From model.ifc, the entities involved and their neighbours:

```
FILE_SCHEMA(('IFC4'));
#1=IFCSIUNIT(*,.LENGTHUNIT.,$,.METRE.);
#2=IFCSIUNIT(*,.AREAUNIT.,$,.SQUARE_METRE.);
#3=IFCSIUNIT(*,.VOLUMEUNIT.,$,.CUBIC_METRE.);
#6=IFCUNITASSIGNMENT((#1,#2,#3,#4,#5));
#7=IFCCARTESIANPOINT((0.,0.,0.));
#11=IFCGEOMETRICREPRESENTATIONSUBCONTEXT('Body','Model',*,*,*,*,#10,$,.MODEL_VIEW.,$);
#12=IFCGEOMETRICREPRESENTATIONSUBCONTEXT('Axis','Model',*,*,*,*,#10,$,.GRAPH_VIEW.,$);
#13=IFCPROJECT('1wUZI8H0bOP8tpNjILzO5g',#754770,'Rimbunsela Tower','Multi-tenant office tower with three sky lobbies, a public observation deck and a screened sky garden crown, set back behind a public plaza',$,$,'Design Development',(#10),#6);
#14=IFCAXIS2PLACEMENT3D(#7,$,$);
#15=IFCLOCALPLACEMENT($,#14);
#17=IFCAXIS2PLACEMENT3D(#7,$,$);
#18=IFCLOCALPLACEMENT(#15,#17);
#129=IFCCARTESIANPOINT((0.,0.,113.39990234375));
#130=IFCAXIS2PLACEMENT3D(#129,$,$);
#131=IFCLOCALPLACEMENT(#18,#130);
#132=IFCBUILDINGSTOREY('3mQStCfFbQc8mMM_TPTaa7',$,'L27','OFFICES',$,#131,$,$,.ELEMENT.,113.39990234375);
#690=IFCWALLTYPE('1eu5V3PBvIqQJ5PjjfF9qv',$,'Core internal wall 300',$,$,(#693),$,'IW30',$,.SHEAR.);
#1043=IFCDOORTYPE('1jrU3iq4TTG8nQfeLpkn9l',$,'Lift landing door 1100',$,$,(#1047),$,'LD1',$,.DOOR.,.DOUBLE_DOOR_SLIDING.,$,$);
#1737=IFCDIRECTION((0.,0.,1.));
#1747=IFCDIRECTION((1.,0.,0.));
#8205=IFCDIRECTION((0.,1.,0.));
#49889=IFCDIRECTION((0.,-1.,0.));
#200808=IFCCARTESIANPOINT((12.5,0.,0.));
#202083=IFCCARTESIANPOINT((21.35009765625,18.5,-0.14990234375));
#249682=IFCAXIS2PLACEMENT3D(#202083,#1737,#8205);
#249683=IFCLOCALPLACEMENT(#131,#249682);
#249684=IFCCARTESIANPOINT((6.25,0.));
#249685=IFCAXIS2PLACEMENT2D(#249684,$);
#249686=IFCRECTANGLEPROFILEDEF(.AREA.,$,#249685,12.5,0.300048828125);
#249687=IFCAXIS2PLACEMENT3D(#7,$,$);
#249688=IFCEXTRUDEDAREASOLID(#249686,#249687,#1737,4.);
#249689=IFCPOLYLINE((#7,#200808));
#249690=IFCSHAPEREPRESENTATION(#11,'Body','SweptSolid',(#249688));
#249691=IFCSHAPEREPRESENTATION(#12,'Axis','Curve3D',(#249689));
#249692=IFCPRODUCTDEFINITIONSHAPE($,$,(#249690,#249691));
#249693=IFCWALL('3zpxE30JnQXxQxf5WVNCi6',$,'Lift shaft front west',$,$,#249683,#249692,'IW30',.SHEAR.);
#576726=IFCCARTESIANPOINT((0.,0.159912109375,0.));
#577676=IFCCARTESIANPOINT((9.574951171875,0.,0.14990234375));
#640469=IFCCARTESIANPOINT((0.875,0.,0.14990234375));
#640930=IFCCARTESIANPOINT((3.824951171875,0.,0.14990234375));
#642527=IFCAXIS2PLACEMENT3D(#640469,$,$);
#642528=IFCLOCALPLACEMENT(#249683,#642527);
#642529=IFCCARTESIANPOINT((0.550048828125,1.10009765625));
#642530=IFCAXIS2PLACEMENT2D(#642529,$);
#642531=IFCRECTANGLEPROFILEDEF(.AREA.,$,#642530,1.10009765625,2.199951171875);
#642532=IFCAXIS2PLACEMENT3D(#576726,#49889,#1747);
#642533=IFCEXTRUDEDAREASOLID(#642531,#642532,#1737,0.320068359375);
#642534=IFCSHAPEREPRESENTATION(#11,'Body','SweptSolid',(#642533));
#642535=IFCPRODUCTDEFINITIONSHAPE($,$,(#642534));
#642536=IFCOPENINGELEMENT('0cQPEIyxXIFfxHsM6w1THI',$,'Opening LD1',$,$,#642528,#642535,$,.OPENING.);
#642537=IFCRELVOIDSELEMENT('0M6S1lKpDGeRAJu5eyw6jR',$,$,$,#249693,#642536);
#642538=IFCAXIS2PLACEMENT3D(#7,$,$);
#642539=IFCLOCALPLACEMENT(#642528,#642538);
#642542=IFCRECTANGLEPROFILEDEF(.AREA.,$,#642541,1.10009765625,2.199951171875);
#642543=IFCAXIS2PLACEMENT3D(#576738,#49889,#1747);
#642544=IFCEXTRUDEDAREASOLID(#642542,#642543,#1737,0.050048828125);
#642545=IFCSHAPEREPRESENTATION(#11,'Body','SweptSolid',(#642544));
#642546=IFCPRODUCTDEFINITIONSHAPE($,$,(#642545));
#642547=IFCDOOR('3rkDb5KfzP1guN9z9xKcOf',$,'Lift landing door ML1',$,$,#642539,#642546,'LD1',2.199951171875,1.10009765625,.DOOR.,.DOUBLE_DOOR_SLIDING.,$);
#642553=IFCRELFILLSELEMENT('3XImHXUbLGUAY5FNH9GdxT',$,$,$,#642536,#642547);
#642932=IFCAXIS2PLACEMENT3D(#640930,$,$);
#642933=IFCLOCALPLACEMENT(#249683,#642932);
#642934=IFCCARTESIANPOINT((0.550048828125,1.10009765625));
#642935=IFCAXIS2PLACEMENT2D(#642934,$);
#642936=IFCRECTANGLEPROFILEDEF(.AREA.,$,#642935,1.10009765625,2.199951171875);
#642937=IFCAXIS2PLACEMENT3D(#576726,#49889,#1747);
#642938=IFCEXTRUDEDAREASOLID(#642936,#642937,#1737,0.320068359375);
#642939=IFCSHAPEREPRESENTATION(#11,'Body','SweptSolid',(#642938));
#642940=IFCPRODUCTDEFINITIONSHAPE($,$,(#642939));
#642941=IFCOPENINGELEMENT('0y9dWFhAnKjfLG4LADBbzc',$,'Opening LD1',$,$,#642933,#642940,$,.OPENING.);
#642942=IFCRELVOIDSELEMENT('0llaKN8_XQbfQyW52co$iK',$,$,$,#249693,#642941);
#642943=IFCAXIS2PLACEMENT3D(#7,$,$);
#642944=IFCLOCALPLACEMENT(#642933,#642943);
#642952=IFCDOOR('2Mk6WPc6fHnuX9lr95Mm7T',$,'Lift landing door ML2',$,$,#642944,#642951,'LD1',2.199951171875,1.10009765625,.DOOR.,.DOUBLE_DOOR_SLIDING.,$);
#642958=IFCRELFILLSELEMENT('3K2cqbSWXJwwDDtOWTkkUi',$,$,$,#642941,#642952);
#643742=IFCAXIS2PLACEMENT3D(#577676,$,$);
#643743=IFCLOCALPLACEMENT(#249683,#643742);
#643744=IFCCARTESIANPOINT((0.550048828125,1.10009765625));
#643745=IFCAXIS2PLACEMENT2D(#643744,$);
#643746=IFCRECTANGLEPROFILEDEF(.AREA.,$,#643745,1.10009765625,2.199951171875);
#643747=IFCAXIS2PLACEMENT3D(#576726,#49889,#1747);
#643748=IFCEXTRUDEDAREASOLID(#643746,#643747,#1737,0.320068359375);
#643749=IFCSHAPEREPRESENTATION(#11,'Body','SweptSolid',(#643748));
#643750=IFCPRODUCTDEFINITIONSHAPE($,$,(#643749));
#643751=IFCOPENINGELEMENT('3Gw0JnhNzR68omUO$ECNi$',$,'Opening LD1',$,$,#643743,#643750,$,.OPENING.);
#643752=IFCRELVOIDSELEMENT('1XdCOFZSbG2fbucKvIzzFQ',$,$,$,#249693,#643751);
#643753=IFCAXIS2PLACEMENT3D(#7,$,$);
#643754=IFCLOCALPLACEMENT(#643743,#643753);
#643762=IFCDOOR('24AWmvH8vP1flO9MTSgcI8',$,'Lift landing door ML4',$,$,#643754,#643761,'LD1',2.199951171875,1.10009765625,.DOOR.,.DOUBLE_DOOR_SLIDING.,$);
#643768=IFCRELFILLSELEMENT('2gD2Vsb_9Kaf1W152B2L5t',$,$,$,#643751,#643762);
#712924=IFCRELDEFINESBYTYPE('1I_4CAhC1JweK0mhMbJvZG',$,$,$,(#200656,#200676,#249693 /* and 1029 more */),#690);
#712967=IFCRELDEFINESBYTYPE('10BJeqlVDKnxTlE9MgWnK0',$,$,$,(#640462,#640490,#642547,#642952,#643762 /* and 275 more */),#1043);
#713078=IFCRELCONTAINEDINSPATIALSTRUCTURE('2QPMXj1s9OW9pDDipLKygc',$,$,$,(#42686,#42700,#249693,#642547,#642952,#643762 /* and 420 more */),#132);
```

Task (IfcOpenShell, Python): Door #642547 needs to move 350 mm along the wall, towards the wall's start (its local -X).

```python
import ifcopenshell
import ifcopenshell.api.geometry
import ifcopenshell.util.placement
import ifcopenshell.util.unit

model = ifcopenshell.open("model.ifc")
unit_scale = ifcopenshell.util.unit.calculate_unit_scale(model)

door = model.by_guid("3rkDb5KfzP1guN9z9xKcOf")
opening = door.FillsVoids[0].RelatingOpeningElement
wall = opening.VoidsElements[0].RelatingBuildingElement

wall_matrix = ifcopenshell.util.placement.get_local_placement(wall.ObjectPlacement)
shift = wall_matrix[:3, 0] * -0.35 / unit_scale
before = ifcopenshell.util.placement.get_local_placement(door.ObjectPlacement)[:3, 3].copy()

# The door is placed relative to its opening, so it follows when the opening moves.
matrix = ifcopenshell.util.placement.get_local_placement(opening.ObjectPlacement)
matrix[:3, 3] += shift
ifcopenshell.api.geometry.edit_object_placement(
    model, product=opening, matrix=matrix, is_si=False, should_transform_children=True
)

after = ifcopenshell.util.placement.get_local_placement(door.ObjectPlacement)[:3, 3]
print("door moved by", (after - before).round(3) + 0.0)

model.write("model_edited.ifc")
```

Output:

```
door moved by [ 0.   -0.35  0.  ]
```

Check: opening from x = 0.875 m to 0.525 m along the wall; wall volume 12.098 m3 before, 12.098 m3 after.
